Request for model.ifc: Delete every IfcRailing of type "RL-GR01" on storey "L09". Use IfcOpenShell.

First a look at what the model holds.

```python
import ifcopenshell
import ifcopenshell.util.element

model = ifcopenshell.open("model.ifc")
print(model.schema)
storey = next(s for s in model.by_type("IfcBuildingStorey") if s.Name == "L09")
railings = [e for e in ifcopenshell.util.element.get_decomposition(storey) if e.is_a("IfcRailing")]
seen = {}
for e in railings:
    element_type = ifcopenshell.util.element.get_type(e)
    name = element_type.Name if element_type not in (None, e) else None
    seen[name] = seen.get(name, 0) + 1
for name, count in sorted(seen.items(), key=str):
    print(count, "x", name)
```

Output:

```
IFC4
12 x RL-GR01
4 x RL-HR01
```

```python
import ifcopenshell
import ifcopenshell.api.root
import ifcopenshell.util.element

model = ifcopenshell.open("model.ifc")

storey = next(s for s in model.by_type("IfcBuildingStorey") if s.Name == "L09")
railings = [e for e in ifcopenshell.util.element.get_decomposition(storey) if e.is_a("IfcRailing")]
targets = [e for e in railings if (t := ifcopenshell.util.element.get_type(e)) not in (None, e) and t.Name == "RL-GR01"]

for e in targets:
    ifcopenshell.api.root.remove_product(model, product=e)
print(len(targets), "removed")

model.write("model_rev.ifc")
```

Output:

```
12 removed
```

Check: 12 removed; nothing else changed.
